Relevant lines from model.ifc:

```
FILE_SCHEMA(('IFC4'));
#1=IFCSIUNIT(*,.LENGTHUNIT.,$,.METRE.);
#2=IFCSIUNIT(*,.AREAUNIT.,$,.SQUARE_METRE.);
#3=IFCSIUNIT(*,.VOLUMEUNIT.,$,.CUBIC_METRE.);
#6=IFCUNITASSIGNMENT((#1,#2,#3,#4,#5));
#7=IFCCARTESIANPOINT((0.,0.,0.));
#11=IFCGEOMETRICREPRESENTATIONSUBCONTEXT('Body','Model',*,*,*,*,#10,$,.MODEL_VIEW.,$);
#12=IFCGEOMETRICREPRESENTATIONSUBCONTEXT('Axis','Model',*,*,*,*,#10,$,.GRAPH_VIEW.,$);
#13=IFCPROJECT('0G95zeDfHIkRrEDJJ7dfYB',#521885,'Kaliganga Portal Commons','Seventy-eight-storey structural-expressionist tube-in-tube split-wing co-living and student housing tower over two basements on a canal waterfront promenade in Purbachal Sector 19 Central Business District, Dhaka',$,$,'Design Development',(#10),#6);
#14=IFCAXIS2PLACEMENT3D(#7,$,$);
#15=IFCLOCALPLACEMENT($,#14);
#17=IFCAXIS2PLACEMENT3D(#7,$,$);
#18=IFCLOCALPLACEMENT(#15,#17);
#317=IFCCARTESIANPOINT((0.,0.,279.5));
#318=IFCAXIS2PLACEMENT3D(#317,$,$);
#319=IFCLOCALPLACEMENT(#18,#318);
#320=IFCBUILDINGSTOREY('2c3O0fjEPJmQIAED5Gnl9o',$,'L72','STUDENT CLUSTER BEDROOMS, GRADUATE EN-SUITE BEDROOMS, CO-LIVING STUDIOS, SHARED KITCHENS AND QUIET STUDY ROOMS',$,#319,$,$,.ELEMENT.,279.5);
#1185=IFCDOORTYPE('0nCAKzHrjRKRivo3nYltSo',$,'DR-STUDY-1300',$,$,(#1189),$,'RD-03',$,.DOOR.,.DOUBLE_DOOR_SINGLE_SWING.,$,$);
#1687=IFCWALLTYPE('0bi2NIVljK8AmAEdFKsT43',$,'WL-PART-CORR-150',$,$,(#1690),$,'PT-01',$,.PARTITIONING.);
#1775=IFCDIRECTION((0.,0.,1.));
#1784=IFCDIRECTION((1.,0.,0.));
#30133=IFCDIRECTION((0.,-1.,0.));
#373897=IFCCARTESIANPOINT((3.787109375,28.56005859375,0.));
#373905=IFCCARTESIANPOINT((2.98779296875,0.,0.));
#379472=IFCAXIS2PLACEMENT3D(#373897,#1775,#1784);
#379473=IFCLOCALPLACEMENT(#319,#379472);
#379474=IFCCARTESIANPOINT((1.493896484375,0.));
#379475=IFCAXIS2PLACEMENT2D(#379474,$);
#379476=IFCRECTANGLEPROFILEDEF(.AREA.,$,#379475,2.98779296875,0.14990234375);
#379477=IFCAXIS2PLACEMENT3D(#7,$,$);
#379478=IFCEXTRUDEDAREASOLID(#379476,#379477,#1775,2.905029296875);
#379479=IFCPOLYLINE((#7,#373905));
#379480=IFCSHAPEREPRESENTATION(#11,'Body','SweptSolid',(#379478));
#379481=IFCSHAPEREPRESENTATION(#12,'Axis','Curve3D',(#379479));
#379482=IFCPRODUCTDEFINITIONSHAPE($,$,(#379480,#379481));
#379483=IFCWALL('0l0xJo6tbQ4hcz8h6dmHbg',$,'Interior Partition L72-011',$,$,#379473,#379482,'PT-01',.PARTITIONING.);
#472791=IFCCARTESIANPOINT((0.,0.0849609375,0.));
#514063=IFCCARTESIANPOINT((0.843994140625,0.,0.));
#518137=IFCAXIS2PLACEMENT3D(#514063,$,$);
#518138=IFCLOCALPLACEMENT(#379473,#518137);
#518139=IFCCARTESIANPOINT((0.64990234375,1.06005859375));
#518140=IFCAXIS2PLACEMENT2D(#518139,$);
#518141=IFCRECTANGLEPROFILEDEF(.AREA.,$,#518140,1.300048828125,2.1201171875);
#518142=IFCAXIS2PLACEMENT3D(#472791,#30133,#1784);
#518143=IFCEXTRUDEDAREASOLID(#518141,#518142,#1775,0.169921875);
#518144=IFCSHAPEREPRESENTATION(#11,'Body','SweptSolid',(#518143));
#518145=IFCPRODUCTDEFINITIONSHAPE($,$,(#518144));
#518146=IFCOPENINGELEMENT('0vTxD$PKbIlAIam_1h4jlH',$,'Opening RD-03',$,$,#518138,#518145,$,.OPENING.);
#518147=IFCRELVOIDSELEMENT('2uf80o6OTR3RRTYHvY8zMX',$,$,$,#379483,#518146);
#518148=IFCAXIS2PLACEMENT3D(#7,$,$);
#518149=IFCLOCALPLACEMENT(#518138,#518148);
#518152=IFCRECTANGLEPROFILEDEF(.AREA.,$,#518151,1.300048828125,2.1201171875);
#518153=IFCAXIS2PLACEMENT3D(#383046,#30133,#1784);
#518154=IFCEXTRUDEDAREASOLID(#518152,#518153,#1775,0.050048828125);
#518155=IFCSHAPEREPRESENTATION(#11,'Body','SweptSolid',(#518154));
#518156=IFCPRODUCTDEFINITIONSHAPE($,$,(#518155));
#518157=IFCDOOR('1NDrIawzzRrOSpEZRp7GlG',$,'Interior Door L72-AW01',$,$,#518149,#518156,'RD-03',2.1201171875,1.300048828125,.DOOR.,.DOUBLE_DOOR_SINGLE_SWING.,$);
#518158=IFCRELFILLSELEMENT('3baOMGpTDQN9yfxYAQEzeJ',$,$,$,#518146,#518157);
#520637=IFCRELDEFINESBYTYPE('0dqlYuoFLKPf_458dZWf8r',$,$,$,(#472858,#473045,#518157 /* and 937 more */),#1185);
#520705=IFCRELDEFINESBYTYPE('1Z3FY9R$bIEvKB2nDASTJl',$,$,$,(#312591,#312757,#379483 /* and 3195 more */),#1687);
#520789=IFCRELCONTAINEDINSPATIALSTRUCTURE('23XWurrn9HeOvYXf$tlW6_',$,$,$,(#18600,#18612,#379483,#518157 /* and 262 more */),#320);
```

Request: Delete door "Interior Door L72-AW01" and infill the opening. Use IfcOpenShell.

```python
import ifcopenshell
import ifcopenshell.api.feature
import ifcopenshell.api.root
import ifcopenshell.geom
import ifcopenshell.util.shape

model = ifcopenshell.open("model.ifc")
settings = ifcopenshell.geom.settings()


def volume(element):
    """Net volume in cubic metres, openings subtracted."""
    shape = ifcopenshell.geom.create_shape(settings, element)
    return ifcopenshell.util.shape.get_volume(shape.geometry)


door = model.by_id(518157)
opening = door.FillsVoids[0].RelatingOpeningElement
wall = opening.VoidsElements[0].RelatingBuildingElement
before = volume(wall)

ifcopenshell.api.root.remove_product(model, product=door)
ifcopenshell.api.feature.remove_feature(model, feature=opening)

after = volume(wall)

print(f"wall volume {before:.3f} -> {after:.3f} m3")

model.write("model_v2.ifc")
```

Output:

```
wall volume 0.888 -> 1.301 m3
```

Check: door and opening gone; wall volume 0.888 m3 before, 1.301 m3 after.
